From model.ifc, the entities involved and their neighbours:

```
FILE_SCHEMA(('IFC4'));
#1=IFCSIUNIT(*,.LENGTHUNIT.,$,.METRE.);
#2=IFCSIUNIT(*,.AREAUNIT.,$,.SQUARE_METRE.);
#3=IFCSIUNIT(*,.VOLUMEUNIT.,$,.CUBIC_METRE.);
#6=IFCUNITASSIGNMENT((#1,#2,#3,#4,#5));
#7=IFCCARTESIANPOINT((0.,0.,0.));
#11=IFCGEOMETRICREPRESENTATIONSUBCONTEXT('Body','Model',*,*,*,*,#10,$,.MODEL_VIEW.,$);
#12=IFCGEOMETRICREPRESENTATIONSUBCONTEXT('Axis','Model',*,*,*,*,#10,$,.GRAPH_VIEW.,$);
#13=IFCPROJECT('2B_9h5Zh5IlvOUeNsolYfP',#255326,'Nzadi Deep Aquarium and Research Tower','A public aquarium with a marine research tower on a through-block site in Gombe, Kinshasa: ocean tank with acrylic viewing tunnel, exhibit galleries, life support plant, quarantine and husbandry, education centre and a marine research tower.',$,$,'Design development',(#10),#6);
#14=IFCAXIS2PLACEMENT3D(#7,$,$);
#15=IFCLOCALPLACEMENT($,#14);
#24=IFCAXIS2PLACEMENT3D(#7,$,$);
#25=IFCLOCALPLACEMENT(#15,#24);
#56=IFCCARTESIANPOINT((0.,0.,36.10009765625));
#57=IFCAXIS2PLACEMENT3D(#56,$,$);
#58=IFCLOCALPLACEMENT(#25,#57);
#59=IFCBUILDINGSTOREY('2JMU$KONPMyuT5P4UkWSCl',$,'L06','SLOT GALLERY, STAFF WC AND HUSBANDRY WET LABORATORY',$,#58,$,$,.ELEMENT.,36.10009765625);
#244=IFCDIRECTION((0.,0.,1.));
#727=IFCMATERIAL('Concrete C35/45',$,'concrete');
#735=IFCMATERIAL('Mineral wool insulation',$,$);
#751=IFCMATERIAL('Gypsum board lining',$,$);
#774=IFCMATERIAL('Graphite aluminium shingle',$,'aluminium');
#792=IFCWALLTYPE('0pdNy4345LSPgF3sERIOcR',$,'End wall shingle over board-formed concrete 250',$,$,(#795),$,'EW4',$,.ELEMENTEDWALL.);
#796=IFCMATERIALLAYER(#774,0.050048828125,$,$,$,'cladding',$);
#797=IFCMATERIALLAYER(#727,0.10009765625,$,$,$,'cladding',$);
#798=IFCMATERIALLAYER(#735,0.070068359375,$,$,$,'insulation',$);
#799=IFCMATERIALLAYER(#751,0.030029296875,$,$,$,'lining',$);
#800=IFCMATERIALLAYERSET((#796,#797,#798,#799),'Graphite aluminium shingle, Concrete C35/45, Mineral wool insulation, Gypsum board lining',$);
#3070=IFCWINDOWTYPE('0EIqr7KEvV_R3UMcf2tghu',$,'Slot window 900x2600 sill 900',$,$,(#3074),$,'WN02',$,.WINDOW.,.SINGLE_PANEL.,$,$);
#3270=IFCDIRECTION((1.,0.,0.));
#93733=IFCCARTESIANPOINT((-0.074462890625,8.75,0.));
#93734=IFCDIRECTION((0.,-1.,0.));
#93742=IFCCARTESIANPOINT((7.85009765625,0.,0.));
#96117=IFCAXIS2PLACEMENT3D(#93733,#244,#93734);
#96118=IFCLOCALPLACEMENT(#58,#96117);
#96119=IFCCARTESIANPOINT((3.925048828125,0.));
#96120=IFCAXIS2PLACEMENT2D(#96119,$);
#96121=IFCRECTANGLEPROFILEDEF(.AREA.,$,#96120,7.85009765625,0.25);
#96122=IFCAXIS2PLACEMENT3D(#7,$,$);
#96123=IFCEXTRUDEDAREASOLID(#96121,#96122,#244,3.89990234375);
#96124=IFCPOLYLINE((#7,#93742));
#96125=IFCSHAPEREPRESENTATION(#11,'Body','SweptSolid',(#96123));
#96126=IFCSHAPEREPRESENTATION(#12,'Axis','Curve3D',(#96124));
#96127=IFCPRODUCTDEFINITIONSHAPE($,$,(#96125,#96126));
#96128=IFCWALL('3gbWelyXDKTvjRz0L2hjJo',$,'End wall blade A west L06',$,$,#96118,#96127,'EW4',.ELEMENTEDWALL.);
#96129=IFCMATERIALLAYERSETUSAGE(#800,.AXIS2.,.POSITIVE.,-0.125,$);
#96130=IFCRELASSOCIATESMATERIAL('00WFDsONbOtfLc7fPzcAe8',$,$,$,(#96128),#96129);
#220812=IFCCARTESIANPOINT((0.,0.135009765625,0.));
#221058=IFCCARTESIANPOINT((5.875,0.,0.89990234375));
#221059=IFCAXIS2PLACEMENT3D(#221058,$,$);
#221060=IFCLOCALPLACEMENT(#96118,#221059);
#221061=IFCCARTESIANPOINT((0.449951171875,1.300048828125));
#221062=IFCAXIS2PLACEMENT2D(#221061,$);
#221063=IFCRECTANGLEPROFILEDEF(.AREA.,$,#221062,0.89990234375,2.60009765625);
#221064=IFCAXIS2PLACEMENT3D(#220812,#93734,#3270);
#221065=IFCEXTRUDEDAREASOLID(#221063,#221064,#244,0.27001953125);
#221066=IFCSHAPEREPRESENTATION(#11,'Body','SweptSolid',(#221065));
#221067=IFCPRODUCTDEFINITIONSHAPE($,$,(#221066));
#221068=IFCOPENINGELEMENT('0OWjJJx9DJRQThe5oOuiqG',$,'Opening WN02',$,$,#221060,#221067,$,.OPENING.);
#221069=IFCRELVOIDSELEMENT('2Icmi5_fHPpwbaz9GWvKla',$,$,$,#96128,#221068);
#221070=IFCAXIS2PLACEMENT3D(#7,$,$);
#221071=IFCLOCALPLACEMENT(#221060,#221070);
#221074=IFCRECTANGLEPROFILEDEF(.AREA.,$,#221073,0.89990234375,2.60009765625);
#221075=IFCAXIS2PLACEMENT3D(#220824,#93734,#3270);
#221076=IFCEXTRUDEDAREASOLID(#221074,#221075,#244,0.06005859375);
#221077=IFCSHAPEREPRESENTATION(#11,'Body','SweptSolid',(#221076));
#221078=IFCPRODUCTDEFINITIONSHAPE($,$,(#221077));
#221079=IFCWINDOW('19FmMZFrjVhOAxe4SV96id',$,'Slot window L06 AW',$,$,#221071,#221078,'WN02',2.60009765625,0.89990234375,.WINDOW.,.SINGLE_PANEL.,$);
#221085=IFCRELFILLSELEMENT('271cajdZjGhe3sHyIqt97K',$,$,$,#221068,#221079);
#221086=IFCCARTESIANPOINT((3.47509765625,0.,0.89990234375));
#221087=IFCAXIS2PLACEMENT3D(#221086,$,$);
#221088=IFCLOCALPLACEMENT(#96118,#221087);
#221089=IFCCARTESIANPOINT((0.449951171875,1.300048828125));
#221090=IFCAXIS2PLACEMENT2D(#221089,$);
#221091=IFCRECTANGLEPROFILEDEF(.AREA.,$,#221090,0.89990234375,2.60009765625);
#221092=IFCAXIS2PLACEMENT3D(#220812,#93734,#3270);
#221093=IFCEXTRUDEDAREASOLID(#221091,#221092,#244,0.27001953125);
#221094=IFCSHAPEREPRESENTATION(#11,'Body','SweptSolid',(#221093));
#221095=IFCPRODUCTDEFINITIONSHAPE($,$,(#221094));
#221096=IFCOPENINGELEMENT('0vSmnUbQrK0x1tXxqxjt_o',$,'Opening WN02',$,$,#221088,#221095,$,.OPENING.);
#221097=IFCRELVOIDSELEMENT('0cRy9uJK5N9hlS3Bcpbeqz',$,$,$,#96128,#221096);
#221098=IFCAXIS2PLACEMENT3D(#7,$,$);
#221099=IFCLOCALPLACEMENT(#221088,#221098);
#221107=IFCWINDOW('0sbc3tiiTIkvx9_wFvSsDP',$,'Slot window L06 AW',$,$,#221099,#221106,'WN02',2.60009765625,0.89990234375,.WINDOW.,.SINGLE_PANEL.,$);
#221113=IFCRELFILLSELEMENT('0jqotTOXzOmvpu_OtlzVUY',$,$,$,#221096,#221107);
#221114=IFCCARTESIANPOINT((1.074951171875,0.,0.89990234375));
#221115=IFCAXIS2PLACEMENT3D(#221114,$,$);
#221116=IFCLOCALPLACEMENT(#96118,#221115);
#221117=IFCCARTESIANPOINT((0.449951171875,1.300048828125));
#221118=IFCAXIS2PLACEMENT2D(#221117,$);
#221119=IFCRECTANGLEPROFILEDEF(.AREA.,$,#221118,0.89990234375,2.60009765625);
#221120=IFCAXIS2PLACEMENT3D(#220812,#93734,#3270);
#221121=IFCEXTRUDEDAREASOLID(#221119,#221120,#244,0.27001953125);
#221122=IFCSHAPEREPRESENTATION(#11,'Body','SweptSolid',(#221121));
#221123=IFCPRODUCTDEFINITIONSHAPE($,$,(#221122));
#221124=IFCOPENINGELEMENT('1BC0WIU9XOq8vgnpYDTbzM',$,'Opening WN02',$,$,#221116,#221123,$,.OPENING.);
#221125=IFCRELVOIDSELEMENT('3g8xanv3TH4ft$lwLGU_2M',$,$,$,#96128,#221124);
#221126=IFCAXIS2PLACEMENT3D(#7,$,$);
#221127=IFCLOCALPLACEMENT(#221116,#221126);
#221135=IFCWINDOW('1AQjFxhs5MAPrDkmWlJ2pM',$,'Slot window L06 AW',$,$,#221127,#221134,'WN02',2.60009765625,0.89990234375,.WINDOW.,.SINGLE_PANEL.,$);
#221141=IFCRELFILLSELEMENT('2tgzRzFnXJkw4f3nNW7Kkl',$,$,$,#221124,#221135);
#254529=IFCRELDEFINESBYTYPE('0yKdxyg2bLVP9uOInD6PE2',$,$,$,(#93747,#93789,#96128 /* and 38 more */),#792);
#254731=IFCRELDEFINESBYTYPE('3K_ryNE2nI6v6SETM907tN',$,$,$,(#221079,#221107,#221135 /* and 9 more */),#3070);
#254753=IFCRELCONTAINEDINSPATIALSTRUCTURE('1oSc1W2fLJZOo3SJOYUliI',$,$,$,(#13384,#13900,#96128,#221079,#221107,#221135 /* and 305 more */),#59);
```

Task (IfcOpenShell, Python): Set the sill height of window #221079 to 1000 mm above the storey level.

```python
import numpy as np
import ifcopenshell
import ifcopenshell.api.geometry
import ifcopenshell.geom
import ifcopenshell.util.element
import ifcopenshell.util.placement
import ifcopenshell.util.shape
import ifcopenshell.util.unit

model = ifcopenshell.open("model.ifc")
unit_scale = ifcopenshell.util.unit.calculate_unit_scale(model)

window = model.by_guid("19FmMZFrjVhOAxe4SV96id")
opening = window.FillsVoids[0].RelatingOpeningElement
storey = ifcopenshell.util.element.get_container(window, ifc_class="IfcBuildingStorey")
level = ifcopenshell.util.placement.get_local_placement(storey.ObjectPlacement)[2, 3]

# The opening's origin need not be at the sill, so measure its lowest point.
shape = ifcopenshell.geom.create_shape(ifcopenshell.geom.settings(), opening)
bottom = ifcopenshell.util.shape.get_shape_bottom_elevation(shape, shape.geometry) / unit_scale
dz = level + 1 / unit_scale - bottom

shift = np.array([0.0, 0.0, dz])
# The window is placed relative to its opening, so it follows when the opening moves.
matrix = ifcopenshell.util.placement.get_local_placement(opening.ObjectPlacement)
matrix[:3, 3] += shift
ifcopenshell.api.geometry.edit_object_placement(
    model, product=opening, matrix=matrix, is_si=False, should_transform_children=True
)

print(f"moved by {dz * unit_scale:+.3f} m")

model.write("model_edited.ifc")
```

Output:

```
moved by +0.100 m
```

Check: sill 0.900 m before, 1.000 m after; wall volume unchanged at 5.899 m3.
